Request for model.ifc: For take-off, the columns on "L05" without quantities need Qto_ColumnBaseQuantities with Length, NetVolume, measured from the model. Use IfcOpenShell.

First a look at what the model holds.

```python
import ifcopenshell
import ifcopenshell.util.element
import ifcopenshell.util.unit

model = ifcopenshell.open("model.ifc")
print(model.schema)
for unit_type in ("LENGTHUNIT", "AREAUNIT", "VOLUMEUNIT"):
    print(unit_type, ifcopenshell.util.unit.calculate_unit_scale(model, unit_type))
storey = next(s for s in model.by_type("IfcBuildingStorey") if s.Name == "L05")
columns = [e for e in ifcopenshell.util.element.get_decomposition(storey) if e.is_a("IfcColumn")]
for e in sorted(columns, key=lambda e: e.id()):
    print(e.id(), e.is_a(), e.Name, list(ifcopenshell.util.element.get_psets(e, qtos_only=True)), sep=" | ")
```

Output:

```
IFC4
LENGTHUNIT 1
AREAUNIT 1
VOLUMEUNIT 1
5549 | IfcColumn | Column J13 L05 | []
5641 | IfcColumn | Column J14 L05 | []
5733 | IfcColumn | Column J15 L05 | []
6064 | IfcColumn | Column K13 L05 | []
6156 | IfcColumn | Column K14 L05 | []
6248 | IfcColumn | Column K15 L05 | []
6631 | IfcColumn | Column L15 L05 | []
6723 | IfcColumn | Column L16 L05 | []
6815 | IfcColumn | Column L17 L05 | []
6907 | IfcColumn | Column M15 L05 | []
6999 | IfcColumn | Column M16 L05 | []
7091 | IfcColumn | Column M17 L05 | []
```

```python
import ifcopenshell
import ifcopenshell.api.pset
import ifcopenshell.geom
import ifcopenshell.util.element
import ifcopenshell.util.shape
import ifcopenshell.util.unit

model = ifcopenshell.open("model.ifc")
unit_scale = ifcopenshell.util.unit.calculate_unit_scale(model)
volume_scale = ifcopenshell.util.unit.calculate_unit_scale(model, "VOLUMEUNIT")
settings = ifcopenshell.geom.settings()

storey = next(s for s in model.by_type("IfcBuildingStorey") if s.Name == "L05")
columns = [e for e in ifcopenshell.util.element.get_decomposition(storey) if e.is_a("IfcColumn")]

for e in sorted(columns, key=lambda e: e.id()):
    if ifcopenshell.util.element.get_psets(e, qtos_only=True, should_inherit=False):
        continue
    # Geometry comes back in metres, in the element's own axes.
    shape = ifcopenshell.geom.create_shape(settings, e)
    values = {
        "Length": ifcopenshell.util.shape.get_z(shape.geometry) / unit_scale,
        "NetVolume": ifcopenshell.util.shape.get_volume(shape.geometry) / volume_scale,
    }
    qto = ifcopenshell.api.pset.add_qto(model, product=e, name="Qto_ColumnBaseQuantities")
    ifcopenshell.api.pset.edit_qto(model, qto=qto, properties=values)
    print(e.id(), {k: round(v, 3) for k, v in values.items()})

model.write("model_updated.ifc")
```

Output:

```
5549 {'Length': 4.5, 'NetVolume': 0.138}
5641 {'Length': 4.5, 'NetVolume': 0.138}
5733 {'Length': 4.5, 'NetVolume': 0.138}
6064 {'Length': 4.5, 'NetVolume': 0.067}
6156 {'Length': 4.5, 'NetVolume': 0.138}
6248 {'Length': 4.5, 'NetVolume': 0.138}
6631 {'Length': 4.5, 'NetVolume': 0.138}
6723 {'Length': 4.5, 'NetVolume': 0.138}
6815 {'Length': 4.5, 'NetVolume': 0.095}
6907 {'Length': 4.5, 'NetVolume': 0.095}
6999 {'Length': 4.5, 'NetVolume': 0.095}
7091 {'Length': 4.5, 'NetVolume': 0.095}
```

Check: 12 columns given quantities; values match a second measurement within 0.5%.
